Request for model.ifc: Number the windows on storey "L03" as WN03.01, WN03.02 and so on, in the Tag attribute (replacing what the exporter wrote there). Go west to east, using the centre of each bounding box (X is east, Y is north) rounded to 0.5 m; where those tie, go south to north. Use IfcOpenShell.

First a look at what the model holds.

```python
import ifcopenshell
import ifcopenshell.util.element
import ifcopenshell.util.placement

model = ifcopenshell.open("model.ifc")
print(model.schema)
storey = next(s for s in model.by_type("IfcBuildingStorey") if s.Name == "L03")
windows = [e for e in ifcopenshell.util.element.get_decomposition(storey) if e.is_a("IfcWindow")]
for e in sorted(windows, key=lambda e: e.id()):
    origin = ifcopenshell.util.placement.get_local_placement(e.ObjectPlacement)[:3, 3]
    print(e.id(), e.Tag, e.Name, origin.round(2) + 0.0, sep=" | ")
```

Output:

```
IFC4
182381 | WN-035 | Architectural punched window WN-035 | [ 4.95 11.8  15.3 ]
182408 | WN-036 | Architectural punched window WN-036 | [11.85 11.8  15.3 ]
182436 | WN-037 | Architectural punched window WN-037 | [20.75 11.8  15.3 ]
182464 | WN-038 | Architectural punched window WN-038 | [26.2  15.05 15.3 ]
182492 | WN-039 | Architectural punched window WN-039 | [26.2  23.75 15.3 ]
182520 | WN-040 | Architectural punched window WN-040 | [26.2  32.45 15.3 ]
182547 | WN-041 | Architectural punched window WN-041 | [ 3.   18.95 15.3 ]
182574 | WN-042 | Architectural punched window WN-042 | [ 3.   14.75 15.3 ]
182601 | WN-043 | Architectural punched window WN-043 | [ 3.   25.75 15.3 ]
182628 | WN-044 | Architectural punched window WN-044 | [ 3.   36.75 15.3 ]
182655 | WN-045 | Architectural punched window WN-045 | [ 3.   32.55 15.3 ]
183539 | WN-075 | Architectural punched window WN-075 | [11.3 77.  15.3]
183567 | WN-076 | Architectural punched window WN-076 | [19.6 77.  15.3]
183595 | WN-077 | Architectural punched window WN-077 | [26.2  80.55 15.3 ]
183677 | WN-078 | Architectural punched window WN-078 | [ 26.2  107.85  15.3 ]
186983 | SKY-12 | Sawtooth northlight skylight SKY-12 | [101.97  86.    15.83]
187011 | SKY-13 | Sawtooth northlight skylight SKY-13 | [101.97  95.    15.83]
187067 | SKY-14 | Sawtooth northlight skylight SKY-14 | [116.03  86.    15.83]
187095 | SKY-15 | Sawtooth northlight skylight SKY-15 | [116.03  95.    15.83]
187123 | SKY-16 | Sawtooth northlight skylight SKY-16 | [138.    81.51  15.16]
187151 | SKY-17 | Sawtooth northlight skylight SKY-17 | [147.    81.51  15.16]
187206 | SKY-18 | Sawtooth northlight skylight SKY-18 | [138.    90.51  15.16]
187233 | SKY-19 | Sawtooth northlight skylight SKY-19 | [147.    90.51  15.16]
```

```python
import ifcopenshell
import ifcopenshell.geom
import ifcopenshell.util.element
import ifcopenshell.util.shape

model = ifcopenshell.open("model.ifc")
settings = ifcopenshell.geom.settings()
settings.set("use-world-coords", True)


def centre(element):
    shape = ifcopenshell.geom.create_shape(settings, element)
    return ifcopenshell.util.shape.get_bbox_centroid(shape.geometry)


storey = next(s for s in model.by_type("IfcBuildingStorey") if s.Name == "L03")
windows = [e for e in ifcopenshell.util.element.get_decomposition(storey) if e.is_a("IfcWindow")]

# Insertion points can sit at a corner or the storey origin, so sort by the geometry (in metres).
centres = {e: centre(e) for e in windows}
windows.sort(key=lambda e: (round(centres[e][0] / 0.5), centres[e][1]))

for i, e in enumerate(windows, start=1):
    number = f"WN03.{i:02d}"
    e.Tag = number
    print(e.id(), number)

model.write("model_edited.ifc")
```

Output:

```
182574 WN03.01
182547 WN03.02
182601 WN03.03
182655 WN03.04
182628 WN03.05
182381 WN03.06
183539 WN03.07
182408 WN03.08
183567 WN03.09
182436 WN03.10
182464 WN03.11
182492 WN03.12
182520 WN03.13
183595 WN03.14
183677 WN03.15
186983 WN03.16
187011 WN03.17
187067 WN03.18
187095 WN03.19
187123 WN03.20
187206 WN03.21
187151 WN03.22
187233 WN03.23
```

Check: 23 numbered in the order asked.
